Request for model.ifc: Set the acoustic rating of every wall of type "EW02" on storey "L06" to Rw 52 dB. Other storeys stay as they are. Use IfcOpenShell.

First a look at what the model holds.

```python
import ifcopenshell
import ifcopenshell.util.element

model = ifcopenshell.open("model.ifc")
print(model.schema)
storey = next(s for s in model.by_type("IfcBuildingStorey") if s.Name == "L06")
walls = [e for e in ifcopenshell.util.element.get_decomposition(storey) if e.is_a("IfcWall")]
seen = {}
for e in walls:
    element_type = ifcopenshell.util.element.get_type(e)
    key = (element_type.Name if element_type != e and element_type else None, ifcopenshell.util.element.get_pset(e, "Pset_WallCommon", "AcousticRating"))
    seen[key] = seen.get(key, 0) + 1
for (name, value), count in sorted(seen.items(), key=str):
    print(count, "x", name, "|", value)
```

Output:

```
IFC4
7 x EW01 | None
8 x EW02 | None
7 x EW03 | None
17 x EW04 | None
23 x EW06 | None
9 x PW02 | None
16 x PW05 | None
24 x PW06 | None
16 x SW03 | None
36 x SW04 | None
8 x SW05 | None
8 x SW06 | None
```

```python
import ifcopenshell
import ifcopenshell.api.pset
import ifcopenshell.util.element

model = ifcopenshell.open("model.ifc")

storey = next(s for s in model.by_type("IfcBuildingStorey") if s.Name == "L06")
walls = [e for e in ifcopenshell.util.element.get_decomposition(storey) if e.is_a("IfcWall")]

count = 0
for e in walls:
    element_type = ifcopenshell.util.element.get_type(e)
    if element_type in (None, e) or element_type.Name != "EW02":
        continue
    # add_pset returns the element's existing set when there is one.
    pset = ifcopenshell.api.pset.add_pset(model, product=e, name="Pset_WallCommon")
    ifcopenshell.api.pset.edit_pset(model, pset=pset, properties={"AcousticRating": "Rw 52 dB"})
    count += 1

print(count, "walls updated")

model.write("model_v2.ifc")
```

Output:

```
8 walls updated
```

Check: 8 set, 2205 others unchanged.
